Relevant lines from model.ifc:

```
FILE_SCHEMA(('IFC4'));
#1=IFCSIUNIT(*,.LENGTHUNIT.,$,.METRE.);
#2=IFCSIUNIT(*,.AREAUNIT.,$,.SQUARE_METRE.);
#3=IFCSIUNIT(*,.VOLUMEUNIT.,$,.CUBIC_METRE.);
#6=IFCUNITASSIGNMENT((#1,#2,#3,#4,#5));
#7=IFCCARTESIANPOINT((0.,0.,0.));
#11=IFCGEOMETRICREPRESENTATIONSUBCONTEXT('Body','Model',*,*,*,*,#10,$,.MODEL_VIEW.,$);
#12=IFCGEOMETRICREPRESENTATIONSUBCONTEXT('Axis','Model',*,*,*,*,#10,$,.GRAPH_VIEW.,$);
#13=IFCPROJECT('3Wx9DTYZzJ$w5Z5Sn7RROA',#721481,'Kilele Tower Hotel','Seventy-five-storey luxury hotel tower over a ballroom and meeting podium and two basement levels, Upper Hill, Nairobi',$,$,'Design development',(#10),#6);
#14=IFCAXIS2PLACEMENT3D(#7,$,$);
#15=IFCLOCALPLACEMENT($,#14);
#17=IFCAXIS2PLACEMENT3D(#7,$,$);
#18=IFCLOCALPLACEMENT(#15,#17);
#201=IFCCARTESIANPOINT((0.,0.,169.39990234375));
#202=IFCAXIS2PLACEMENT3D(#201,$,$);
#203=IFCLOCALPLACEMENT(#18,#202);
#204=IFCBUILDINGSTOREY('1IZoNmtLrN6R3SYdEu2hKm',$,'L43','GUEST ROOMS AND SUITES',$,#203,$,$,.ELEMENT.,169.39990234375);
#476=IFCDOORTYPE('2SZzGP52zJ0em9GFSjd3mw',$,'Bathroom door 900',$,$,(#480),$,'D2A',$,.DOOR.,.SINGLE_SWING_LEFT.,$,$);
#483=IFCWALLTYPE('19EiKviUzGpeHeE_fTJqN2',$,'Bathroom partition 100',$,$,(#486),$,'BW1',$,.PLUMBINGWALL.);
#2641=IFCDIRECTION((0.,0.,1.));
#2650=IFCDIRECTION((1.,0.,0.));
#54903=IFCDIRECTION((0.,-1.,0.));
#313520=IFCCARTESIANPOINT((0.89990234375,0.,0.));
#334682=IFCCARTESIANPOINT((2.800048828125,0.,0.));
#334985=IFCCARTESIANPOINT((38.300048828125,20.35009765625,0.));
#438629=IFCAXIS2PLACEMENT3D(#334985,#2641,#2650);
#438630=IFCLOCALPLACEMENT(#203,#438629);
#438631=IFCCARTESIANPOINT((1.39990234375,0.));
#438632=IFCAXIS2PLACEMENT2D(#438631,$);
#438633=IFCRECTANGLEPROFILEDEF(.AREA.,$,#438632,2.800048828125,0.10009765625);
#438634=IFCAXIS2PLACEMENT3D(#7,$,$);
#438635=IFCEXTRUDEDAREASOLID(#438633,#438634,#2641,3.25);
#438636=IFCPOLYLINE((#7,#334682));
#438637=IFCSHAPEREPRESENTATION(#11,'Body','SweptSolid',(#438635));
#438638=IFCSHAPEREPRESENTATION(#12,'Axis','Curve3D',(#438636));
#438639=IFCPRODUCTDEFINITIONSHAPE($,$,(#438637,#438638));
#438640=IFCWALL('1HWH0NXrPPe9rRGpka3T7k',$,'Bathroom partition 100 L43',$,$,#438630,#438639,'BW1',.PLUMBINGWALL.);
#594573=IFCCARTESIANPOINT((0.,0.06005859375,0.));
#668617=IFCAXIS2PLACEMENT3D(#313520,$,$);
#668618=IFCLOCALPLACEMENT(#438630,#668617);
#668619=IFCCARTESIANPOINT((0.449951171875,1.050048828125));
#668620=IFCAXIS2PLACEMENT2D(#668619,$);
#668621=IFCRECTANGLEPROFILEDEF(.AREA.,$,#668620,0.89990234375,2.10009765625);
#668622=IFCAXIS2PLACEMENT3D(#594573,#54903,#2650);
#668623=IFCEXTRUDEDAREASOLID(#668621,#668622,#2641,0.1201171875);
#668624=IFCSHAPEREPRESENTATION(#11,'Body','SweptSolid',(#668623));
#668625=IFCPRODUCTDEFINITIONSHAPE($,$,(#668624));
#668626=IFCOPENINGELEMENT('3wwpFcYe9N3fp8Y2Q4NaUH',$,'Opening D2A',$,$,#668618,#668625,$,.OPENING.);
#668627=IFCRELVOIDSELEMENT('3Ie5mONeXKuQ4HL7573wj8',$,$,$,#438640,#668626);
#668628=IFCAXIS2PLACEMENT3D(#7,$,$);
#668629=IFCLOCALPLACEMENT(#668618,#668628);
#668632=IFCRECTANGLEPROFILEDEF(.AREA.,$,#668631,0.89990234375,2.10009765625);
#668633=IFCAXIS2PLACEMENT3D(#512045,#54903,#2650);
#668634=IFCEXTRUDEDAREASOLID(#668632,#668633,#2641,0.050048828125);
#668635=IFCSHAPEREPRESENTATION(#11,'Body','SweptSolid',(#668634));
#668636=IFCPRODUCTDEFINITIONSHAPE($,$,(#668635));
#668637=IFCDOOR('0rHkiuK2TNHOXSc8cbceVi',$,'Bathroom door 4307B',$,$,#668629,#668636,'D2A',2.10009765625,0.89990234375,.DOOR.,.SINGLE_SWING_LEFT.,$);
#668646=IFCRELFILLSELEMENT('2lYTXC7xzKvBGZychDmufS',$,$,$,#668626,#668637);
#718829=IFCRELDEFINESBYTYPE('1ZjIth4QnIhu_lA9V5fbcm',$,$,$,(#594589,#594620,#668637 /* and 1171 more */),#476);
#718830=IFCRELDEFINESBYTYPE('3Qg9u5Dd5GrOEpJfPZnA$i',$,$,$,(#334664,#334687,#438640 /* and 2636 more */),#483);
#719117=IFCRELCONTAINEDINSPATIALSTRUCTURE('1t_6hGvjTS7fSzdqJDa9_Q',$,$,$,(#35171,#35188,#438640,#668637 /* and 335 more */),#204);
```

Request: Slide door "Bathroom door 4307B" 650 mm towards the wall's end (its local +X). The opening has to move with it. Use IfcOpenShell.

```python
import ifcopenshell
import ifcopenshell.api.geometry
import ifcopenshell.util.placement

model = ifcopenshell.open("model.ifc")

door = model.by_guid("0rHkiuK2TNHOXSc8cbceVi")
opening = door.FillsVoids[0].RelatingOpeningElement
wall = opening.VoidsElements[0].RelatingBuildingElement

wall_matrix = ifcopenshell.util.placement.get_local_placement(wall.ObjectPlacement)
shift = wall_matrix[:3, 0] * 0.65
before = ifcopenshell.util.placement.get_local_placement(door.ObjectPlacement)[:3, 3].copy()

# The door is placed relative to its opening, so it follows when the opening moves.
matrix = ifcopenshell.util.placement.get_local_placement(opening.ObjectPlacement)
matrix[:3, 3] += shift
ifcopenshell.api.geometry.edit_object_placement(
    model, product=opening, matrix=matrix, is_si=False, should_transform_children=True
)

after = ifcopenshell.util.placement.get_local_placement(door.ObjectPlacement)[:3, 3]
print("door moved by", (after - before).round(3) + 0.0)

model.write("model_rev.ifc")
```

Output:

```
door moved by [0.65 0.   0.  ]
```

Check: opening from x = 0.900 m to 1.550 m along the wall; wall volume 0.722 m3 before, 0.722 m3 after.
